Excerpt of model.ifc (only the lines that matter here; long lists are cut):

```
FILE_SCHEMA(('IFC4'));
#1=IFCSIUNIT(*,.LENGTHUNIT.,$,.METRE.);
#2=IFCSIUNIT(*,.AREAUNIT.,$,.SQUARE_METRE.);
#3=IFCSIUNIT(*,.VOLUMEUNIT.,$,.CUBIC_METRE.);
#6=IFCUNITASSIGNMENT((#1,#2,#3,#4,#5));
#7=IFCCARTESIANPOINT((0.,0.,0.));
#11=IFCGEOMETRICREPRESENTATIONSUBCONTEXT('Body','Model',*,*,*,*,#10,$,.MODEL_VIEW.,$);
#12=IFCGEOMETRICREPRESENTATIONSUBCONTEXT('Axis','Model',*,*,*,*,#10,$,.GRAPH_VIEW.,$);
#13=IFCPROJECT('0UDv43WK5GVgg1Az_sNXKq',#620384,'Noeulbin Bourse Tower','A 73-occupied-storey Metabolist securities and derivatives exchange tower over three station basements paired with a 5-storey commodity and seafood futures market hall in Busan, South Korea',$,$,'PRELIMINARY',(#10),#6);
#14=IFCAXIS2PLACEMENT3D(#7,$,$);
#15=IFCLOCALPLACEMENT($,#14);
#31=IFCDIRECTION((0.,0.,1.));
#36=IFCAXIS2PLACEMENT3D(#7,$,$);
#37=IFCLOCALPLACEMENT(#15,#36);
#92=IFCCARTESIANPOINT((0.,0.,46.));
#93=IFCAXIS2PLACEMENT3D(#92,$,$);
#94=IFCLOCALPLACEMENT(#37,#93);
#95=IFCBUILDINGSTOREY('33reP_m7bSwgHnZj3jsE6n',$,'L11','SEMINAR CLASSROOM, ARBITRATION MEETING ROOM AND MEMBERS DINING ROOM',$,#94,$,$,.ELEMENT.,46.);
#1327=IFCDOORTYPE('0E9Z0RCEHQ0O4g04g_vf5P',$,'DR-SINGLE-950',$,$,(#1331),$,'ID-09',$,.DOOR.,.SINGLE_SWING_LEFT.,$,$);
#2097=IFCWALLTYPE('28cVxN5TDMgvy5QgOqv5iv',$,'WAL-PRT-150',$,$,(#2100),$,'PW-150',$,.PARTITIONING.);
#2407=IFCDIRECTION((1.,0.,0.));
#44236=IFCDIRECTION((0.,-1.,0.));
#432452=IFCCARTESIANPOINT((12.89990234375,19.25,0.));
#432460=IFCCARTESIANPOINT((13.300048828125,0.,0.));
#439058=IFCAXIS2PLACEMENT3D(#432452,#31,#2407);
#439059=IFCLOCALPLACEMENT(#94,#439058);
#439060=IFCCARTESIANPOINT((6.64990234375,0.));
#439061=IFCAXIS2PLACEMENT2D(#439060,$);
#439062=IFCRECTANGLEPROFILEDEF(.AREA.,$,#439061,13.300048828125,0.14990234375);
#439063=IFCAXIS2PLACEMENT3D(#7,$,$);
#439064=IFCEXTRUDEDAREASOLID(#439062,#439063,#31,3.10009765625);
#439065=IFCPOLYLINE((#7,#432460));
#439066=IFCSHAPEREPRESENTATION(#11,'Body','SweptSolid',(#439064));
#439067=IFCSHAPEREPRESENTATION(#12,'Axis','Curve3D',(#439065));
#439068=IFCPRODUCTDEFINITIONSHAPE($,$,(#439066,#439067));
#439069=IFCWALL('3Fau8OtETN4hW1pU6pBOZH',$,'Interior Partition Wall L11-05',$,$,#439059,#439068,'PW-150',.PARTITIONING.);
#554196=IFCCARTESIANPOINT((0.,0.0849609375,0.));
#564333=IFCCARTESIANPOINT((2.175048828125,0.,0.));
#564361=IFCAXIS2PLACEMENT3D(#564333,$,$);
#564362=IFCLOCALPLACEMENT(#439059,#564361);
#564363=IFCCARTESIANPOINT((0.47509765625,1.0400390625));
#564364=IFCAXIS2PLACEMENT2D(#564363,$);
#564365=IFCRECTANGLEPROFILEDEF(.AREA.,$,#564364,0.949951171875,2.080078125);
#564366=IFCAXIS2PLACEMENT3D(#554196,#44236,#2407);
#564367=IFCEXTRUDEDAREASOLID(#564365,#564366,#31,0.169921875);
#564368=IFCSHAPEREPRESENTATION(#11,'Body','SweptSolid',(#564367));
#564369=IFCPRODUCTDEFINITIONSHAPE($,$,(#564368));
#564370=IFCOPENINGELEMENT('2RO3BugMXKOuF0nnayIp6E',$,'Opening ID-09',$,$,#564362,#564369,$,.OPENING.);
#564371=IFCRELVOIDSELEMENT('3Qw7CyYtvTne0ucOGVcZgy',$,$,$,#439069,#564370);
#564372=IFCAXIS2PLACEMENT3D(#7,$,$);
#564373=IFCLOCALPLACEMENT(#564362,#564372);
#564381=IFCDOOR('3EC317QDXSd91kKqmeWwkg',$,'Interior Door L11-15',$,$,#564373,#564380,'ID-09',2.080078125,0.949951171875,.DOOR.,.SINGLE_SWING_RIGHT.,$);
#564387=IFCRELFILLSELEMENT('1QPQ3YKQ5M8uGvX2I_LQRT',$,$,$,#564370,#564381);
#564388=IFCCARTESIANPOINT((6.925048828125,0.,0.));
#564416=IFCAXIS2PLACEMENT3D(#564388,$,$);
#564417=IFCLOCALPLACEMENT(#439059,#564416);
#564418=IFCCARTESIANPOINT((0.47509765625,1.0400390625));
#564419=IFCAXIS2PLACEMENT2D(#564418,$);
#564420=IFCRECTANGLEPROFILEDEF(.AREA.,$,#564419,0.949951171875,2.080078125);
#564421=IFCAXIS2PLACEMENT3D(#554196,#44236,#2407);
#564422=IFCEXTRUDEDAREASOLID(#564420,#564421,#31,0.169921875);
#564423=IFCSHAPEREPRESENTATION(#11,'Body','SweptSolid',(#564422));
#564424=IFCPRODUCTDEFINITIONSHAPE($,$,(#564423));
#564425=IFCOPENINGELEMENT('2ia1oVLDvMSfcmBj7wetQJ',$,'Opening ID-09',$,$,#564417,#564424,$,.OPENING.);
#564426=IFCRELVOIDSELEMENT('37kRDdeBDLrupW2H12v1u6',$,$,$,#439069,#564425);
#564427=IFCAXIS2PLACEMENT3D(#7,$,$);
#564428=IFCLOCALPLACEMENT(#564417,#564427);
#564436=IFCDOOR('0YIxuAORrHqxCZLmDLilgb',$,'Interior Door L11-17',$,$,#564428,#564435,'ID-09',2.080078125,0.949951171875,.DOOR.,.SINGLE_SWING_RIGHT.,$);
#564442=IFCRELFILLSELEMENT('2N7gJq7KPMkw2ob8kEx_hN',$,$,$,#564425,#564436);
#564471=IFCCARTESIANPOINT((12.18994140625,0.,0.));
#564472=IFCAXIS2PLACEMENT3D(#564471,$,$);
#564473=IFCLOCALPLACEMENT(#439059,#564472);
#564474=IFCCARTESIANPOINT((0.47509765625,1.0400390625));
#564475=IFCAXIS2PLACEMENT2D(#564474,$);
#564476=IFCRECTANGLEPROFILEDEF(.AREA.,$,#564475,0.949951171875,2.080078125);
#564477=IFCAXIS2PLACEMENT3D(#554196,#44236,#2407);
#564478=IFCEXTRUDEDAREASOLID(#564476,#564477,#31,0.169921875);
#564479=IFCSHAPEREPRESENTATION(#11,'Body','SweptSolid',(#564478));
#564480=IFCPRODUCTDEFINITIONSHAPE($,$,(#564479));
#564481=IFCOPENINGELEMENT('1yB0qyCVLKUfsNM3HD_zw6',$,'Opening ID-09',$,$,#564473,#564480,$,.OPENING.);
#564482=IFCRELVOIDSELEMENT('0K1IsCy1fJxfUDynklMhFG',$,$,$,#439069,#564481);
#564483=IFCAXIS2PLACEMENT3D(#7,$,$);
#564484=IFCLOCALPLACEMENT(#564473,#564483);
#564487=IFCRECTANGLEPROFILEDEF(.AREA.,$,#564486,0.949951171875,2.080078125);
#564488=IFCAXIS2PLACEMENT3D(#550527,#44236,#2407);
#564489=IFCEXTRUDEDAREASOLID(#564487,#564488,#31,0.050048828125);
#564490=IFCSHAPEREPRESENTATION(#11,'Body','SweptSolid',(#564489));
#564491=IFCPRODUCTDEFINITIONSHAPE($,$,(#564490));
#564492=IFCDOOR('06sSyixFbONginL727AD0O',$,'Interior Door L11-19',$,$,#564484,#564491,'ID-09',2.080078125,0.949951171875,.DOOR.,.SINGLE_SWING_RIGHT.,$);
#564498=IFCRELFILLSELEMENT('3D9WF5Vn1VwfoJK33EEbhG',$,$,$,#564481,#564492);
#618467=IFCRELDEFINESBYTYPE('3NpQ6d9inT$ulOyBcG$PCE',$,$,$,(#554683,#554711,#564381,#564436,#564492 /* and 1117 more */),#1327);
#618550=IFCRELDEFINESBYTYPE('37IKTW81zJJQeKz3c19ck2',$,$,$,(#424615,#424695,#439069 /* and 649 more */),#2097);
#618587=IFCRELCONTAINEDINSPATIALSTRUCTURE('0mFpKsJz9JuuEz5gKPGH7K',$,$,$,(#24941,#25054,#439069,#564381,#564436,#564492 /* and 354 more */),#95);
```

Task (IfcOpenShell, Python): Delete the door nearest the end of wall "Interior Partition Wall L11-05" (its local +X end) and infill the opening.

```python
import ifcopenshell
import ifcopenshell.api.feature
import ifcopenshell.api.root
import ifcopenshell.geom
import ifcopenshell.util.shape

model = ifcopenshell.open("model.ifc")
settings = ifcopenshell.geom.settings()


def volume(element):
    """Net volume in cubic metres, openings subtracted."""
    shape = ifcopenshell.geom.create_shape(settings, element)
    return ifcopenshell.util.shape.get_volume(shape.geometry)


door = model.by_id(564492)
opening = door.FillsVoids[0].RelatingOpeningElement
wall = opening.VoidsElements[0].RelatingBuildingElement
before = volume(wall)

ifcopenshell.api.root.remove_product(model, product=door)
ifcopenshell.api.feature.remove_feature(model, feature=opening)

after = volume(wall)

print(f"wall volume {before:.3f} -> {after:.3f} m3")

model.write("model_rev.ifc")
```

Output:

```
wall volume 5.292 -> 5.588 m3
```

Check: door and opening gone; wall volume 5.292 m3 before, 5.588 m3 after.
